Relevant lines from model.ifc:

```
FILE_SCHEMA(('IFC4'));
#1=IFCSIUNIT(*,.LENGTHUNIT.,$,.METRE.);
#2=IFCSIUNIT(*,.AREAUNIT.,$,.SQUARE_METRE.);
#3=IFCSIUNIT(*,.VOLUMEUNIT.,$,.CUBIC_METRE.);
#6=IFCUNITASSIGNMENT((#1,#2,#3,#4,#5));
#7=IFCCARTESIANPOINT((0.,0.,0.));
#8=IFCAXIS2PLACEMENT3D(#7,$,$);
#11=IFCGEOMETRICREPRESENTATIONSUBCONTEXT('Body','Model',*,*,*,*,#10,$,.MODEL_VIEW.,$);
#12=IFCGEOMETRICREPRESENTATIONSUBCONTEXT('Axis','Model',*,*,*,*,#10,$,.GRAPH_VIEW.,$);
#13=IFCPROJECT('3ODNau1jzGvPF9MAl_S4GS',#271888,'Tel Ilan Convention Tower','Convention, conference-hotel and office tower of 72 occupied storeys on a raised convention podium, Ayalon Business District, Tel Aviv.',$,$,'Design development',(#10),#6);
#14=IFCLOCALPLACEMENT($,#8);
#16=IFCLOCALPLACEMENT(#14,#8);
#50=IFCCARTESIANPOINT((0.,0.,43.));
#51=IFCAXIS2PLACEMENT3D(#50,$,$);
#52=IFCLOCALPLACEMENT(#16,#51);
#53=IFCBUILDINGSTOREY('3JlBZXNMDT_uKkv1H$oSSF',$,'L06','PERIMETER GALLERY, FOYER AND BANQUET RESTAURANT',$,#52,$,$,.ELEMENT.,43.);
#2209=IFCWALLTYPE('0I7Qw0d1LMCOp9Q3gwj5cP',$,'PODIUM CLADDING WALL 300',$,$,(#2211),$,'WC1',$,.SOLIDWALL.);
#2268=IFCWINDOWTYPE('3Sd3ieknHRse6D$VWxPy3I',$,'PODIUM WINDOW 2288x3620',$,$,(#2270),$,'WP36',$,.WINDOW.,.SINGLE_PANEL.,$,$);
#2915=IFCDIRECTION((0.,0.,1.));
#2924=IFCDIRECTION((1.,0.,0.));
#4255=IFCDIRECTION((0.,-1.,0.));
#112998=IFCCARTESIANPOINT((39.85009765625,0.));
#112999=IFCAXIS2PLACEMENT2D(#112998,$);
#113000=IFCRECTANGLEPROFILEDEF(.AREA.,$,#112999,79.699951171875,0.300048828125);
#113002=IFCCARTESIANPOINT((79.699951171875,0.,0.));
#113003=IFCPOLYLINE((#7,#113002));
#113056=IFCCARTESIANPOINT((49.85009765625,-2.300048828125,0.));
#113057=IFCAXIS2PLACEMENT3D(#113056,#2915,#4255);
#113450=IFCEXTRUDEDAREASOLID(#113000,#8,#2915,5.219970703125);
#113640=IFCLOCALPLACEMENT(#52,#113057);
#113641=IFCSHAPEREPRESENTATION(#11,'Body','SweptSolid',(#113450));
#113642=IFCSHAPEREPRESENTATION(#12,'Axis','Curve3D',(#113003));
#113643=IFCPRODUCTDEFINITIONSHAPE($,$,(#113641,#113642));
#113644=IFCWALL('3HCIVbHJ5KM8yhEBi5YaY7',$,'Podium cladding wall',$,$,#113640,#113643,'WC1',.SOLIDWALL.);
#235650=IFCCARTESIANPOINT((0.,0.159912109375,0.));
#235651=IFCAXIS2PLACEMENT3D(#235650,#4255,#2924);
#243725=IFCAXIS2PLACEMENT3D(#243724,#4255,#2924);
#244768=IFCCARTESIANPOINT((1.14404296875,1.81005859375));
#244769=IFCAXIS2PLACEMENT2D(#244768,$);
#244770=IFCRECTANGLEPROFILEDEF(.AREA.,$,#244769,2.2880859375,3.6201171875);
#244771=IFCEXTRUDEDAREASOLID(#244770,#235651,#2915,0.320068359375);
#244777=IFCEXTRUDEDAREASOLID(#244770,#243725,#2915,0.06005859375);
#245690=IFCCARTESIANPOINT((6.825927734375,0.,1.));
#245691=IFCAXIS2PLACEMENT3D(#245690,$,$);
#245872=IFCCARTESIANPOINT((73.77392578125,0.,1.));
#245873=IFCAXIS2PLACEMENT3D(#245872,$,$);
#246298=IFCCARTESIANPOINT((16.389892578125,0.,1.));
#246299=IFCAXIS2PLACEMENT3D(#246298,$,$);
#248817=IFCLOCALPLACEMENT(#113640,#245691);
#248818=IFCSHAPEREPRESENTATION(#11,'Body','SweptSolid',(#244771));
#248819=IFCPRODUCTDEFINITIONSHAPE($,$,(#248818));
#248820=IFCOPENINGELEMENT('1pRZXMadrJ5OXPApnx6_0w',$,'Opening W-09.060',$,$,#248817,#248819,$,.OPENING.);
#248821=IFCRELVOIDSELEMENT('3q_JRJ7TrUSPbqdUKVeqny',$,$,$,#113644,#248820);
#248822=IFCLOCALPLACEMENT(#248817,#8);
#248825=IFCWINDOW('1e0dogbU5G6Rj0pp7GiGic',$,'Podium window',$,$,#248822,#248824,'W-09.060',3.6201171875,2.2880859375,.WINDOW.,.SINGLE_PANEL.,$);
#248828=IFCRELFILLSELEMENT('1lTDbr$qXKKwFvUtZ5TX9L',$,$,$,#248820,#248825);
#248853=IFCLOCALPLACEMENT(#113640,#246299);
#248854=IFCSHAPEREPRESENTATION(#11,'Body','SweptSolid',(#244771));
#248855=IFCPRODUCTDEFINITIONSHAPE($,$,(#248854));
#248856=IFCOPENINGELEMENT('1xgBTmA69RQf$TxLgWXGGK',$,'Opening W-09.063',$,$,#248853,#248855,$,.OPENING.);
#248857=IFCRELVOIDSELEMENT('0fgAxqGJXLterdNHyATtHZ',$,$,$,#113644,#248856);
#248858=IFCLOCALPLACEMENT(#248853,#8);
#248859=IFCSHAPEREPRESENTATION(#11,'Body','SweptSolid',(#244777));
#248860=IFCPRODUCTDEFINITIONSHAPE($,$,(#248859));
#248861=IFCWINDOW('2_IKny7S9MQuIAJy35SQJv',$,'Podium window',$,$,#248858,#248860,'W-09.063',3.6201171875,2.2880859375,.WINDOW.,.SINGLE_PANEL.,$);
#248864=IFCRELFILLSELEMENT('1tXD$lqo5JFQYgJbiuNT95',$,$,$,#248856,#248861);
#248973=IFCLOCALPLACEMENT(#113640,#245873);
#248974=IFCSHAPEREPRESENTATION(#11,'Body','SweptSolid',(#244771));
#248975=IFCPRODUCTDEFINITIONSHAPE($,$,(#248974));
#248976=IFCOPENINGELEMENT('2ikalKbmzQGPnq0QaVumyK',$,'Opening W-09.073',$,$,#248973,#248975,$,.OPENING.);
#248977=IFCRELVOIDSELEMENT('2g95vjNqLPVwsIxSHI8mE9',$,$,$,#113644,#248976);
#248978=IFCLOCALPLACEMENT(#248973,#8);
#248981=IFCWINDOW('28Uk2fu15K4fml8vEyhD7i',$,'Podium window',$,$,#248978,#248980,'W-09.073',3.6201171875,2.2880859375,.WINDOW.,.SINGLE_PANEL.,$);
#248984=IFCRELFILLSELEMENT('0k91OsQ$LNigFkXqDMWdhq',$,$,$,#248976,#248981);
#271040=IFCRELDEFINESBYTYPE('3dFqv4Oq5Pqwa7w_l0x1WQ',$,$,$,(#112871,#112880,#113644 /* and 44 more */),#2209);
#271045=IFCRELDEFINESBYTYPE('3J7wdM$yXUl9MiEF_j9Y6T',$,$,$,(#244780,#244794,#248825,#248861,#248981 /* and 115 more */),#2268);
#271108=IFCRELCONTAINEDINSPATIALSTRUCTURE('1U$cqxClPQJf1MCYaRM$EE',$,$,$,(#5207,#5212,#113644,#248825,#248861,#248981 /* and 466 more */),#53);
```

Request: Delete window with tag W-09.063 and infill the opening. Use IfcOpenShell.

```python
import ifcopenshell
import ifcopenshell.api.feature
import ifcopenshell.api.root
import ifcopenshell.geom
import ifcopenshell.util.shape

model = ifcopenshell.open("model.ifc")
settings = ifcopenshell.geom.settings()


def volume(element):
    """Net volume in cubic metres, openings subtracted."""
    shape = ifcopenshell.geom.create_shape(settings, element)
    return ifcopenshell.util.shape.get_volume(shape.geometry)


window = model.by_id(248861)
opening = window.FillsVoids[0].RelatingOpeningElement
wall = opening.VoidsElements[0].RelatingBuildingElement
before = volume(wall)

ifcopenshell.api.root.remove_product(model, product=window)
ifcopenshell.api.feature.remove_feature(model, feature=opening)

after = volume(wall)

print(f"wall volume {before:.3f} -> {after:.3f} m3")

model.write("model_edited.ifc")
```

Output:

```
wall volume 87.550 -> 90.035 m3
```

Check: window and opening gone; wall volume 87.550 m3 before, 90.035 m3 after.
